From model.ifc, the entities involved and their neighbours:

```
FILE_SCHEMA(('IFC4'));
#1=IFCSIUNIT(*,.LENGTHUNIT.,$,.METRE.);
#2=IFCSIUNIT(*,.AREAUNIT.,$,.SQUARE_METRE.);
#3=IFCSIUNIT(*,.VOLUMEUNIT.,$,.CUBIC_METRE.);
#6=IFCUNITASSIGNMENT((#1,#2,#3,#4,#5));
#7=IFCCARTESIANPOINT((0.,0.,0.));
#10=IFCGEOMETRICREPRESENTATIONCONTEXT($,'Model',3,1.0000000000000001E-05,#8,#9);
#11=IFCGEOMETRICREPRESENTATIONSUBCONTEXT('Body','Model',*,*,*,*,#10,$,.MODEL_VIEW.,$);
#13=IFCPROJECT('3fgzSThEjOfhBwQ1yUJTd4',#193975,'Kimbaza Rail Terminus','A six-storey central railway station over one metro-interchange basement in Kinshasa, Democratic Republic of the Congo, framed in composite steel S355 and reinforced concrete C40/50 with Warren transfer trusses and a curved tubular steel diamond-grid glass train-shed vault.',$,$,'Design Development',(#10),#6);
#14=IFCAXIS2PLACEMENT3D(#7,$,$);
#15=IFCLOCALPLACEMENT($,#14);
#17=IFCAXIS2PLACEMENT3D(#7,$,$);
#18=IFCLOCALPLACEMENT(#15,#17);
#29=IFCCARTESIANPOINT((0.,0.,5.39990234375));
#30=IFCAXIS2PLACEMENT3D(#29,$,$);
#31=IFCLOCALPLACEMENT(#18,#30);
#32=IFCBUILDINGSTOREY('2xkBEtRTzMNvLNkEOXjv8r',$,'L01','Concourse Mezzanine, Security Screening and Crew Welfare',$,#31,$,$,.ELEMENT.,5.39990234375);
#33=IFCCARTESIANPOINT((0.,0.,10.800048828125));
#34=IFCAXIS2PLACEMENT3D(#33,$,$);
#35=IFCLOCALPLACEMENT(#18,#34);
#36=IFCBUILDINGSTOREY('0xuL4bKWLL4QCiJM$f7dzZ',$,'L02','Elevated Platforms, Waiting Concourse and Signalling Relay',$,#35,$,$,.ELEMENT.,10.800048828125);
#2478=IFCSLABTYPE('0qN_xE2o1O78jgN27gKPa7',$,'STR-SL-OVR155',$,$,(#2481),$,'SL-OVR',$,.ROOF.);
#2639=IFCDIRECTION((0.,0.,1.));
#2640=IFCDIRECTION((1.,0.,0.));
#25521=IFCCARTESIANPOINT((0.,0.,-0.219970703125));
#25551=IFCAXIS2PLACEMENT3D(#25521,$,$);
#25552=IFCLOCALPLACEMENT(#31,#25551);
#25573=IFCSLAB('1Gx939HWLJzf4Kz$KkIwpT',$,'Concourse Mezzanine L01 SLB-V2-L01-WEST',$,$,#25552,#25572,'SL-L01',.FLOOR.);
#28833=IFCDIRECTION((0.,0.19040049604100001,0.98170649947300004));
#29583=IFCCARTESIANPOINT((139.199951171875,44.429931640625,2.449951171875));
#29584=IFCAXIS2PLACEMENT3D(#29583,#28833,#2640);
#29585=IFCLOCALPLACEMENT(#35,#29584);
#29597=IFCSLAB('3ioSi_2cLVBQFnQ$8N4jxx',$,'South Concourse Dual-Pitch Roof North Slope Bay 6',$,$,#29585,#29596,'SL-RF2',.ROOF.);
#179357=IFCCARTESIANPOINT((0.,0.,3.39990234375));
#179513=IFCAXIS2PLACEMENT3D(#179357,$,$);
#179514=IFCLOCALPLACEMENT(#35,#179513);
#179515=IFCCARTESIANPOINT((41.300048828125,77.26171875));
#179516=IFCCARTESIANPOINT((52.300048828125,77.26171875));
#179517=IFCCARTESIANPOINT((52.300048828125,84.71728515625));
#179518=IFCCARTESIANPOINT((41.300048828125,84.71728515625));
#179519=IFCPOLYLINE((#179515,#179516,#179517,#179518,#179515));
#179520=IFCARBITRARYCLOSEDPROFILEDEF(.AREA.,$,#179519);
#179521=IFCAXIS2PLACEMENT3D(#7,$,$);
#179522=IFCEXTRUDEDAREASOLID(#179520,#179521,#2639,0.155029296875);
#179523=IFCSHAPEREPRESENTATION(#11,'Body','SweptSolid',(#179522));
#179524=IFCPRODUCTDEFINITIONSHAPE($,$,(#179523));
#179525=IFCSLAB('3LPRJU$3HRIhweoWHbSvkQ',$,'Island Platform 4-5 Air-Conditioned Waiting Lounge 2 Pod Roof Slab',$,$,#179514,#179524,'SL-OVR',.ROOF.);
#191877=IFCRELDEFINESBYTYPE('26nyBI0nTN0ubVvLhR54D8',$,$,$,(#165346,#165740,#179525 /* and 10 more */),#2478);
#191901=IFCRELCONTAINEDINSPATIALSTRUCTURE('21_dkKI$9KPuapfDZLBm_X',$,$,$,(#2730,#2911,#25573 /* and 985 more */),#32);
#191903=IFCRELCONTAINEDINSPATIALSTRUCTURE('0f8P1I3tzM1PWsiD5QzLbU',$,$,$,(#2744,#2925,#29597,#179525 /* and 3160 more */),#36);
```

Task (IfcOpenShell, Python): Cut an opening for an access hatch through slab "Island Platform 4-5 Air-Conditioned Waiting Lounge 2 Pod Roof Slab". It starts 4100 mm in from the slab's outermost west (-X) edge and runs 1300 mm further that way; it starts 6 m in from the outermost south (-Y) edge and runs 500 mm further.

```python
import numpy as np
import ifcopenshell
import ifcopenshell.api.feature
import ifcopenshell.api.geometry
import ifcopenshell.api.root
import ifcopenshell.geom
import ifcopenshell.util.placement
import ifcopenshell.util.representation
import ifcopenshell.util.shape
import ifcopenshell.util.unit

model = ifcopenshell.open("model.ifc")
unit_scale = ifcopenshell.util.unit.calculate_unit_scale(model)
settings = ifcopenshell.geom.settings()


def volume(element):
    """Net volume in cubic metres, openings subtracted."""
    shape = ifcopenshell.geom.create_shape(settings, element)
    return ifcopenshell.util.shape.get_volume(shape.geometry)


slab = model.by_guid("3LPRJU$3HRIhweoWHbSvkQ")
before = volume(slab)

# Extent in the slab's own axes, in metres. The edges named are its -X and -Y sides.
slab_shape = ifcopenshell.geom.create_shape(settings, slab)
vertices = ifcopenshell.util.shape.get_vertices(slab_shape.geometry)
x_min, y_min, bottom = vertices.min(axis=0)
top = vertices[:, 2].max()

opening = ifcopenshell.api.root.create_entity(model, ifc_class="IfcOpeningElement", name="Access hatch opening", predefined_type="OPENING")
context = ifcopenshell.util.representation.get_context(model, "Model", "Body", "MODEL_VIEW")
width, depth = 1.3, 0.5
outline = [(0.0, 0.0), (width, 0.0), (width, depth), (0.0, depth), (0.0, 0.0)]
# Overshoot both faces by 50 mm so the cut is clean.
shape = ifcopenshell.api.geometry.add_slab_representation(
    model, context=context, depth=top - bottom + 0.1, polyline=outline
)
ifcopenshell.api.geometry.assign_representation(model, product=opening, representation=shape)

matrix = ifcopenshell.util.placement.get_local_placement(slab.ObjectPlacement)
matrix[:, 3] = matrix @ np.append(np.array([x_min + 4.1, y_min + 6, bottom - 0.05]) / unit_scale, 1.0)
ifcopenshell.api.geometry.edit_object_placement(model, product=opening, matrix=matrix, is_si=False)
ifcopenshell.api.feature.add_feature(model, feature=opening, element=slab)

after = volume(slab)

print(f"slab volume {before:.3f} -> {after:.3f} m3")

model.write("model-out.ifc")
```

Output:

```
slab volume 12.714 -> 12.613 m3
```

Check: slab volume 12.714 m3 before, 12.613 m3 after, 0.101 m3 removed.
